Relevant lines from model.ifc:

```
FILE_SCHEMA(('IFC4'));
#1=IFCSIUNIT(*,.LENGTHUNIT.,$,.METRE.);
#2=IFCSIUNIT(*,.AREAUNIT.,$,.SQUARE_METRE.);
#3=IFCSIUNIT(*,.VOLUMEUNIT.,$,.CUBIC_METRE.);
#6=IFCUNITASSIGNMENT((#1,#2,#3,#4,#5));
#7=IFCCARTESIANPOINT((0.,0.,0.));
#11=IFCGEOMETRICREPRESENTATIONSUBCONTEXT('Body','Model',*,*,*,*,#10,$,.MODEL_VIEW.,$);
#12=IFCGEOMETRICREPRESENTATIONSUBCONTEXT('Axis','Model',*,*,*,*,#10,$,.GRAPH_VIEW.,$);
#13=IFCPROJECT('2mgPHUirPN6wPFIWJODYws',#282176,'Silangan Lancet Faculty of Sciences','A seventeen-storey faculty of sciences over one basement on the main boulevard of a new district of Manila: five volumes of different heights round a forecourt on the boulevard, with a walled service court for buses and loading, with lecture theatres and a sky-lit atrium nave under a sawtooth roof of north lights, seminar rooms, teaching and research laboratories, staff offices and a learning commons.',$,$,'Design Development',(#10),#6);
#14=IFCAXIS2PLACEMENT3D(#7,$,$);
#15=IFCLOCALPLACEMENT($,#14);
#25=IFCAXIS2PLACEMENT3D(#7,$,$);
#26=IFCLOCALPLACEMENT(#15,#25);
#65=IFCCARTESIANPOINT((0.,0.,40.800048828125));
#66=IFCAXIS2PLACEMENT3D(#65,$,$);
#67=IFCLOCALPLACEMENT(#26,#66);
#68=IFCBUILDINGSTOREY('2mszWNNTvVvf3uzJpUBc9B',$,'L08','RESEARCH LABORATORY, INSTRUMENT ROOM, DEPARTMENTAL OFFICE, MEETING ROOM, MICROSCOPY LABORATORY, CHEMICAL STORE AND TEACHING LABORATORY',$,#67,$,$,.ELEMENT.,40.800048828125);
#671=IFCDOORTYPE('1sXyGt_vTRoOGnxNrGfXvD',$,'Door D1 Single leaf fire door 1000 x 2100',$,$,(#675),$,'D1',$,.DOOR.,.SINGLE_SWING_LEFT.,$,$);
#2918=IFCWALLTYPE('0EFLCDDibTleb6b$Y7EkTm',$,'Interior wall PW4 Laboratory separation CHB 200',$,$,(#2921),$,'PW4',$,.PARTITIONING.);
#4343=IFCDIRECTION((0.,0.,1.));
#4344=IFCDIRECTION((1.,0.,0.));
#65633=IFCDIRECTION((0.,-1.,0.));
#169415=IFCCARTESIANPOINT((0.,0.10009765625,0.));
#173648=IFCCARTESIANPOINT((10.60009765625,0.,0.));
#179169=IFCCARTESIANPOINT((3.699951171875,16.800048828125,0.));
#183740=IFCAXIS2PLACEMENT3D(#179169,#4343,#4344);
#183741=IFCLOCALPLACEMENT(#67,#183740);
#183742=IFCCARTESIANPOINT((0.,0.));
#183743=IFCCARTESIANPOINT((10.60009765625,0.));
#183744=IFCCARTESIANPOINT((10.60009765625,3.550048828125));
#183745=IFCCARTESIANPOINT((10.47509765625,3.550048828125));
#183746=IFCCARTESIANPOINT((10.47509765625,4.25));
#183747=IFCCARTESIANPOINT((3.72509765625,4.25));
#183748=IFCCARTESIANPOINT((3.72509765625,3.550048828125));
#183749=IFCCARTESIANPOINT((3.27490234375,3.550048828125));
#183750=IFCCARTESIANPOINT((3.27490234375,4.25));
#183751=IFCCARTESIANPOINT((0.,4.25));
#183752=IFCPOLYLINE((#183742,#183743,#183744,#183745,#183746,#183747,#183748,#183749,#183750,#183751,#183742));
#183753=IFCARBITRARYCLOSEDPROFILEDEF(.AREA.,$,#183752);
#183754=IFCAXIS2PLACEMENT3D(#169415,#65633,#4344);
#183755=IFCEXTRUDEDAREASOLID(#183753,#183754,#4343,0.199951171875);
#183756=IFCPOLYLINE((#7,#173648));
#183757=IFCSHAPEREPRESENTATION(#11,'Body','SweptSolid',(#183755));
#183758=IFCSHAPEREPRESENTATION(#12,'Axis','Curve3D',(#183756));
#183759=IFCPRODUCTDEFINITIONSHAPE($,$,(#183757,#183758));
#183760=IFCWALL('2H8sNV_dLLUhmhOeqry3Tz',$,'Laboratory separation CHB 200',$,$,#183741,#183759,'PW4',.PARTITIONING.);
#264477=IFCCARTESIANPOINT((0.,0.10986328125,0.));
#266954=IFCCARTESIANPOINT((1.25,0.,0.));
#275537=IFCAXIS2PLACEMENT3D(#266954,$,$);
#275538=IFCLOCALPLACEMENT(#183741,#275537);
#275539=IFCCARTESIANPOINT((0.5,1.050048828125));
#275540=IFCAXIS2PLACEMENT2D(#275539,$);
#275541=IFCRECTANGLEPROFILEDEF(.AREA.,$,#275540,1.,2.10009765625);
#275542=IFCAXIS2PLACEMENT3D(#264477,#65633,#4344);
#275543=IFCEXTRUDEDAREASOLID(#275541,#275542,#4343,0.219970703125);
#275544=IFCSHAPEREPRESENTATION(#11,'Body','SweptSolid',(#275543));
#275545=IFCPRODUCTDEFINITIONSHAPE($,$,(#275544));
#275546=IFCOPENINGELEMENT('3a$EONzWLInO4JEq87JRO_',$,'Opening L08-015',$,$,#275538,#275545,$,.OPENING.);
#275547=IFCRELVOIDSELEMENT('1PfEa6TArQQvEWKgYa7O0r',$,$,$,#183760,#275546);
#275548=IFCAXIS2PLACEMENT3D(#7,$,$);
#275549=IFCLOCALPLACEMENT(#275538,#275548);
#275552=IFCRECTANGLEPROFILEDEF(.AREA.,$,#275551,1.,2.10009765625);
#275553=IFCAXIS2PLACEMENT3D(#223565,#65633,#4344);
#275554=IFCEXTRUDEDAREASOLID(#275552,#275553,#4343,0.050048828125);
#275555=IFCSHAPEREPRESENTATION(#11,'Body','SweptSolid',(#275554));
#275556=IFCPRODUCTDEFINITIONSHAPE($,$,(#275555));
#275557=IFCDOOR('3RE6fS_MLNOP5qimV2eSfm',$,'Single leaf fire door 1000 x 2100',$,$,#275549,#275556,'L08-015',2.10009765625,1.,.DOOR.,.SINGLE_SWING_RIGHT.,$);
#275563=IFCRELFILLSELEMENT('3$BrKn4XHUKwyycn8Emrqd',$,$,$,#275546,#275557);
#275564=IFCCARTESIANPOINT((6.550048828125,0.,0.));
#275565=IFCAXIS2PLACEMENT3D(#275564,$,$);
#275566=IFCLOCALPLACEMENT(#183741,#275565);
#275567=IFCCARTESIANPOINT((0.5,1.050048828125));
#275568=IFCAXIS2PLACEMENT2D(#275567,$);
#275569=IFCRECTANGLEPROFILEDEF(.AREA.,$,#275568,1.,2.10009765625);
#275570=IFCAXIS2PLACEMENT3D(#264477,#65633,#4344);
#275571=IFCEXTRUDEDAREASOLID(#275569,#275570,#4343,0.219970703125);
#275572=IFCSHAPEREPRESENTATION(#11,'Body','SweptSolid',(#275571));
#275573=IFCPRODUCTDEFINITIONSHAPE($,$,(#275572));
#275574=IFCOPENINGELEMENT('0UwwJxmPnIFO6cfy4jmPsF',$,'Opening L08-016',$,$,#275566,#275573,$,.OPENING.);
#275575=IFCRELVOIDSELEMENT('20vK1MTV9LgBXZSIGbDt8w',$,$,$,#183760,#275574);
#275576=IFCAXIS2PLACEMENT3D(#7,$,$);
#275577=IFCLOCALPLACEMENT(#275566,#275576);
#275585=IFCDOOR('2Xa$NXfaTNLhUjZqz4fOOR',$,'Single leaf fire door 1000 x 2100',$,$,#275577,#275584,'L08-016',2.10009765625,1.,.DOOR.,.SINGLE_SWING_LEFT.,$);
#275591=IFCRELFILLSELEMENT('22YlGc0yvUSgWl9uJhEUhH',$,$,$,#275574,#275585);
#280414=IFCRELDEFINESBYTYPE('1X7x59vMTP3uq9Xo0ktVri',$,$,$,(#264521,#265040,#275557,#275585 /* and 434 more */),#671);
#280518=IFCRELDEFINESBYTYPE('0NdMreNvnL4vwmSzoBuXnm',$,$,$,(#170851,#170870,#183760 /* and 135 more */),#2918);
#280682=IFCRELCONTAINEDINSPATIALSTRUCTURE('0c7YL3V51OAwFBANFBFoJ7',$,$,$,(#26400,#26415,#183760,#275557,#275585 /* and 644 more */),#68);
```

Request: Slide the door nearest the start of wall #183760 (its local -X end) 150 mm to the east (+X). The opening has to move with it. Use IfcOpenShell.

```python
import ifcopenshell
import ifcopenshell.api.geometry
import ifcopenshell.util.placement
import ifcopenshell.util.unit

model = ifcopenshell.open("model.ifc")
unit_scale = ifcopenshell.util.unit.calculate_unit_scale(model)

door = model.by_id(275557)
opening = door.FillsVoids[0].RelatingOpeningElement
wall = opening.VoidsElements[0].RelatingBuildingElement

wall_matrix = ifcopenshell.util.placement.get_local_placement(wall.ObjectPlacement)
shift = wall_matrix[:3, 0] * 0.15 / unit_scale
before = ifcopenshell.util.placement.get_local_placement(door.ObjectPlacement)[:3, 3].copy()

# The door is placed relative to its opening, so it follows when the opening moves.
matrix = ifcopenshell.util.placement.get_local_placement(opening.ObjectPlacement)
matrix[:3, 3] += shift
ifcopenshell.api.geometry.edit_object_placement(
    model, product=opening, matrix=matrix, is_si=False, should_transform_children=True
)

after = ifcopenshell.util.placement.get_local_placement(door.ObjectPlacement)[:3, 3]
print("door moved by", (after - before).round(3) + 0.0)

model.write("model-out.ifc")
```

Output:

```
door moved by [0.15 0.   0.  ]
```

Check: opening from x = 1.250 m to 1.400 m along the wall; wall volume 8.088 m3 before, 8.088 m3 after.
